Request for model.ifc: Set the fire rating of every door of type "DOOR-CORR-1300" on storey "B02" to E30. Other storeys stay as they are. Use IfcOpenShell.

First a look at what the model holds.

```python
import ifcopenshell
import ifcopenshell.util.element

model = ifcopenshell.open("model.ifc")
print(model.schema)
storey = next(s for s in model.by_type("IfcBuildingStorey") if s.Name == "B02")
doors = [e for e in ifcopenshell.util.element.get_decomposition(storey) if e.is_a("IfcDoor")]
seen = {}
for e in doors:
    element_type = ifcopenshell.util.element.get_type(e)
    key = (element_type.Name if element_type != e and element_type else None, ifcopenshell.util.element.get_pset(e, "Pset_DoorCommon", "FireRating"))
    seen[key] = seen.get(key, 0) + 1
for (name, value), count in sorted(seen.items(), key=str):
    print(count, "x", name, "|", value)
```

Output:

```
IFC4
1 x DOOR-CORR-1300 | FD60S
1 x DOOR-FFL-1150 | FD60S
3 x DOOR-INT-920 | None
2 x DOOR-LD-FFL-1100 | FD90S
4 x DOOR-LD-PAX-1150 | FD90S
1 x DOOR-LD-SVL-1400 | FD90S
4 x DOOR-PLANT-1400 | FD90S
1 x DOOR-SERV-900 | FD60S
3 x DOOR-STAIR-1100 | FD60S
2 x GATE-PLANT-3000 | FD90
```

```python
import ifcopenshell
import ifcopenshell.api.pset
import ifcopenshell.util.element

model = ifcopenshell.open("model.ifc")

storey = next(s for s in model.by_type("IfcBuildingStorey") if s.Name == "B02")
doors = [e for e in ifcopenshell.util.element.get_decomposition(storey) if e.is_a("IfcDoor")]

count = 0
for e in doors:
    element_type = ifcopenshell.util.element.get_type(e)
    if element_type in (None, e) or element_type.Name != "DOOR-CORR-1300":
        continue
    # add_pset returns the element's existing set when there is one.
    pset = ifcopenshell.api.pset.add_pset(model, product=e, name="Pset_DoorCommon")
    ifcopenshell.api.pset.edit_pset(model, pset=pset, properties={"FireRating": "E30"})
    count += 1

print(count, "doors updated")

model.write("model_updated.ifc")
```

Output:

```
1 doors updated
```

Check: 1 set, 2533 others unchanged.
